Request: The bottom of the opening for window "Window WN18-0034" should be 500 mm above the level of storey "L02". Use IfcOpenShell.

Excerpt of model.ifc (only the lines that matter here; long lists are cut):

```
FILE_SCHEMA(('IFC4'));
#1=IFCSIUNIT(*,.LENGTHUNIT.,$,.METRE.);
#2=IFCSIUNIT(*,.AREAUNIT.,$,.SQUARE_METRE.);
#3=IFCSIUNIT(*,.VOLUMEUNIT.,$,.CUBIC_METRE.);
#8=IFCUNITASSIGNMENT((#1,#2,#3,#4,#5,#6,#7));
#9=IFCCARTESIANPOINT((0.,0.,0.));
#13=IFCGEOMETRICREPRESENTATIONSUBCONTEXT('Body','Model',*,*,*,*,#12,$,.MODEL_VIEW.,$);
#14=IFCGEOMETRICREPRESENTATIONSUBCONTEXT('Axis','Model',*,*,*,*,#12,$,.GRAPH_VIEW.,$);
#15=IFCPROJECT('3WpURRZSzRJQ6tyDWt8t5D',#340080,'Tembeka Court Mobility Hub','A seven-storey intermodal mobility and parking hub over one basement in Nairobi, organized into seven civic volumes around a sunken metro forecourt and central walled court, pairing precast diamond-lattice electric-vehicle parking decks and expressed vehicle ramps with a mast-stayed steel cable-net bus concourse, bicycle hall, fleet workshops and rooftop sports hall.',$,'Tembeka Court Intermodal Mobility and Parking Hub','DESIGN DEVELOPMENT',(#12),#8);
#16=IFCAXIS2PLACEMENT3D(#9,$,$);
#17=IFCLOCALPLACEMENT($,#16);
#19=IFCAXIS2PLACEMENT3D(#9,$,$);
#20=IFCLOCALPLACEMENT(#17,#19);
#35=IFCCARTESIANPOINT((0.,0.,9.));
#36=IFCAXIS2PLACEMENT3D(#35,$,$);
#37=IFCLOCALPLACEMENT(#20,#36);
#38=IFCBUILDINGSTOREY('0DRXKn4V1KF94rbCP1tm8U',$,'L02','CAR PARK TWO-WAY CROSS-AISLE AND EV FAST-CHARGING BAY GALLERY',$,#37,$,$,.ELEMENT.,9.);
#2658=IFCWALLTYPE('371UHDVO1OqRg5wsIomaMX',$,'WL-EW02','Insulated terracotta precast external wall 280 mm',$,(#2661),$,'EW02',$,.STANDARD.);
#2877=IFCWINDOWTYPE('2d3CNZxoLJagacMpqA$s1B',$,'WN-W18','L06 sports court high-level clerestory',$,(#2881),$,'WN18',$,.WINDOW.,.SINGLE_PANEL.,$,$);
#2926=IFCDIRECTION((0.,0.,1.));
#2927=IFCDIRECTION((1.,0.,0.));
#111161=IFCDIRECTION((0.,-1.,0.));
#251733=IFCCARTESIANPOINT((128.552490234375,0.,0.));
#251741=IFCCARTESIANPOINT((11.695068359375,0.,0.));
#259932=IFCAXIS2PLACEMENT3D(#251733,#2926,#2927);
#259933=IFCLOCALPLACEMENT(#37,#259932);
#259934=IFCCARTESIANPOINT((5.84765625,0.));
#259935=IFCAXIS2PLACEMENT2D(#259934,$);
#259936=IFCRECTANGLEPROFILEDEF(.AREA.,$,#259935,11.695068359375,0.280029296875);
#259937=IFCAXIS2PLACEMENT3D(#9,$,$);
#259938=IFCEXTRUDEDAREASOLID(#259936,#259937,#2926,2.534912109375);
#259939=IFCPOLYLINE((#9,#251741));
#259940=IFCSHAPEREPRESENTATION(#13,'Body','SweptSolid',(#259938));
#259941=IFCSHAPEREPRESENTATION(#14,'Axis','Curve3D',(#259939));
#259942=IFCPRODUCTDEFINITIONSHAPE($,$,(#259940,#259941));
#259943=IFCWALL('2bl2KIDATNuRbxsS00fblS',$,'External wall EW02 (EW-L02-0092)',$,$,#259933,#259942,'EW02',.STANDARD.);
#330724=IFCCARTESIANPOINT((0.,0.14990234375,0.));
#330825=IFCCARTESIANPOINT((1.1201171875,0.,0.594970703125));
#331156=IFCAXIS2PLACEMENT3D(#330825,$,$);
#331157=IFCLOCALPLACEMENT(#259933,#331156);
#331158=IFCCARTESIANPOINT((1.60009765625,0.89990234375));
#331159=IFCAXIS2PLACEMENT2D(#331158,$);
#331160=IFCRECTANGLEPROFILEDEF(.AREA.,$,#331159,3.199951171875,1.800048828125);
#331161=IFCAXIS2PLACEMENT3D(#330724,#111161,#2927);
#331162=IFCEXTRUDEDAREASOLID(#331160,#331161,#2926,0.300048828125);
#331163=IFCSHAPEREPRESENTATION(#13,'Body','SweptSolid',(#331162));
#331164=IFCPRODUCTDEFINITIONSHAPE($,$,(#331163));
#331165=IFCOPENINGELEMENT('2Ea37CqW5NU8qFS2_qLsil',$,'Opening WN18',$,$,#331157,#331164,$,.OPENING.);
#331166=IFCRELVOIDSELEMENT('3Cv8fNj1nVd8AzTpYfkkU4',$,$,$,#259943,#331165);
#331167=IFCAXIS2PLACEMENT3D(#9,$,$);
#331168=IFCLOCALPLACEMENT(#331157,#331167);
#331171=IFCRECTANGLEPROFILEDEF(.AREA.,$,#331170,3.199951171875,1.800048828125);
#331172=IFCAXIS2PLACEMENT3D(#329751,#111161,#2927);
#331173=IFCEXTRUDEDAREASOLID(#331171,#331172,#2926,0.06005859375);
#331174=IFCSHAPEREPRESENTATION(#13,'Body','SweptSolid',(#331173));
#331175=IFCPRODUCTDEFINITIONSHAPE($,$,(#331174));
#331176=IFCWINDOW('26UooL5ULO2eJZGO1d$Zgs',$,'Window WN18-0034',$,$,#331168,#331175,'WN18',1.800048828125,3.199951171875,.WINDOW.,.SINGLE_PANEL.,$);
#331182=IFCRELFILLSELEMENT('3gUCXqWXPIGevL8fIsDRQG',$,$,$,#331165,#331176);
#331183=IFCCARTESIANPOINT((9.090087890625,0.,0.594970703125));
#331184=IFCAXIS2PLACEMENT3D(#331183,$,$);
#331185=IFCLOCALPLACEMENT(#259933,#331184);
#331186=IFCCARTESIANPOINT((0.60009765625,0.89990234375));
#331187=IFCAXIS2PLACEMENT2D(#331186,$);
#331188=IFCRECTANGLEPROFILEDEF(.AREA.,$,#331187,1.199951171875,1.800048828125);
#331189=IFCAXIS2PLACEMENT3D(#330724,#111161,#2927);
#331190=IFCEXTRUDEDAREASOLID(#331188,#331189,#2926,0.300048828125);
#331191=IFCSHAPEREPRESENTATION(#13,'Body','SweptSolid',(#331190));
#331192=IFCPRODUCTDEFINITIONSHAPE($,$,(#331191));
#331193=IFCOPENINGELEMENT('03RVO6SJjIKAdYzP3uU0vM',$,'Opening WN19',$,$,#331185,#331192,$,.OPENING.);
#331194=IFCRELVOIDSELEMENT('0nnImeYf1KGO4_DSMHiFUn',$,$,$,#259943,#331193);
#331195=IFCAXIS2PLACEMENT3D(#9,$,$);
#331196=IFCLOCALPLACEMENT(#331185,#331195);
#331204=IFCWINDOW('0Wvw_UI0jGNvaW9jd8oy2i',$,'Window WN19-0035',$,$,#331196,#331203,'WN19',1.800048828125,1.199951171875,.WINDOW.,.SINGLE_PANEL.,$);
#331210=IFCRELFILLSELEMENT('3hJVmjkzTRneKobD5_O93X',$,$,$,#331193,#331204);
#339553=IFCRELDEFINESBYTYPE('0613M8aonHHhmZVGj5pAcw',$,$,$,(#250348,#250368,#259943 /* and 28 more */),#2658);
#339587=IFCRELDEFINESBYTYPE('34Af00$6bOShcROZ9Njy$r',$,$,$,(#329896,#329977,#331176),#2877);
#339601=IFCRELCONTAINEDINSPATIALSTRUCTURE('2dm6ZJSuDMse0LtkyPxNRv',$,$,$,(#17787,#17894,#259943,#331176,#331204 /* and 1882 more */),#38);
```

```python
import numpy as np
import ifcopenshell
import ifcopenshell.api.geometry
import ifcopenshell.geom
import ifcopenshell.util.element
import ifcopenshell.util.placement
import ifcopenshell.util.shape
import ifcopenshell.util.unit

model = ifcopenshell.open("model.ifc")
unit_scale = ifcopenshell.util.unit.calculate_unit_scale(model)

window = model.by_guid("26UooL5ULO2eJZGO1d$Zgs")
opening = window.FillsVoids[0].RelatingOpeningElement
storey = ifcopenshell.util.element.get_container(window, ifc_class="IfcBuildingStorey")
level = ifcopenshell.util.placement.get_local_placement(storey.ObjectPlacement)[2, 3]

# The opening's origin need not be at the sill, so measure its lowest point.
shape = ifcopenshell.geom.create_shape(ifcopenshell.geom.settings(), opening)
bottom = ifcopenshell.util.shape.get_shape_bottom_elevation(shape, shape.geometry) / unit_scale
dz = level + 0.5 - bottom

shift = np.array([0.0, 0.0, dz])
# The window is placed relative to its opening, so it follows when the opening moves.
matrix = ifcopenshell.util.placement.get_local_placement(opening.ObjectPlacement)
matrix[:3, 3] += shift
ifcopenshell.api.geometry.edit_object_placement(
    model, product=opening, matrix=matrix, is_si=False, should_transform_children=True
)

print(f"moved by {dz * unit_scale:+.3f} m")

model.write("model_updated.ifc")
```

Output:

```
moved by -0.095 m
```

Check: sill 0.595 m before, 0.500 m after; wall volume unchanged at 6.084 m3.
